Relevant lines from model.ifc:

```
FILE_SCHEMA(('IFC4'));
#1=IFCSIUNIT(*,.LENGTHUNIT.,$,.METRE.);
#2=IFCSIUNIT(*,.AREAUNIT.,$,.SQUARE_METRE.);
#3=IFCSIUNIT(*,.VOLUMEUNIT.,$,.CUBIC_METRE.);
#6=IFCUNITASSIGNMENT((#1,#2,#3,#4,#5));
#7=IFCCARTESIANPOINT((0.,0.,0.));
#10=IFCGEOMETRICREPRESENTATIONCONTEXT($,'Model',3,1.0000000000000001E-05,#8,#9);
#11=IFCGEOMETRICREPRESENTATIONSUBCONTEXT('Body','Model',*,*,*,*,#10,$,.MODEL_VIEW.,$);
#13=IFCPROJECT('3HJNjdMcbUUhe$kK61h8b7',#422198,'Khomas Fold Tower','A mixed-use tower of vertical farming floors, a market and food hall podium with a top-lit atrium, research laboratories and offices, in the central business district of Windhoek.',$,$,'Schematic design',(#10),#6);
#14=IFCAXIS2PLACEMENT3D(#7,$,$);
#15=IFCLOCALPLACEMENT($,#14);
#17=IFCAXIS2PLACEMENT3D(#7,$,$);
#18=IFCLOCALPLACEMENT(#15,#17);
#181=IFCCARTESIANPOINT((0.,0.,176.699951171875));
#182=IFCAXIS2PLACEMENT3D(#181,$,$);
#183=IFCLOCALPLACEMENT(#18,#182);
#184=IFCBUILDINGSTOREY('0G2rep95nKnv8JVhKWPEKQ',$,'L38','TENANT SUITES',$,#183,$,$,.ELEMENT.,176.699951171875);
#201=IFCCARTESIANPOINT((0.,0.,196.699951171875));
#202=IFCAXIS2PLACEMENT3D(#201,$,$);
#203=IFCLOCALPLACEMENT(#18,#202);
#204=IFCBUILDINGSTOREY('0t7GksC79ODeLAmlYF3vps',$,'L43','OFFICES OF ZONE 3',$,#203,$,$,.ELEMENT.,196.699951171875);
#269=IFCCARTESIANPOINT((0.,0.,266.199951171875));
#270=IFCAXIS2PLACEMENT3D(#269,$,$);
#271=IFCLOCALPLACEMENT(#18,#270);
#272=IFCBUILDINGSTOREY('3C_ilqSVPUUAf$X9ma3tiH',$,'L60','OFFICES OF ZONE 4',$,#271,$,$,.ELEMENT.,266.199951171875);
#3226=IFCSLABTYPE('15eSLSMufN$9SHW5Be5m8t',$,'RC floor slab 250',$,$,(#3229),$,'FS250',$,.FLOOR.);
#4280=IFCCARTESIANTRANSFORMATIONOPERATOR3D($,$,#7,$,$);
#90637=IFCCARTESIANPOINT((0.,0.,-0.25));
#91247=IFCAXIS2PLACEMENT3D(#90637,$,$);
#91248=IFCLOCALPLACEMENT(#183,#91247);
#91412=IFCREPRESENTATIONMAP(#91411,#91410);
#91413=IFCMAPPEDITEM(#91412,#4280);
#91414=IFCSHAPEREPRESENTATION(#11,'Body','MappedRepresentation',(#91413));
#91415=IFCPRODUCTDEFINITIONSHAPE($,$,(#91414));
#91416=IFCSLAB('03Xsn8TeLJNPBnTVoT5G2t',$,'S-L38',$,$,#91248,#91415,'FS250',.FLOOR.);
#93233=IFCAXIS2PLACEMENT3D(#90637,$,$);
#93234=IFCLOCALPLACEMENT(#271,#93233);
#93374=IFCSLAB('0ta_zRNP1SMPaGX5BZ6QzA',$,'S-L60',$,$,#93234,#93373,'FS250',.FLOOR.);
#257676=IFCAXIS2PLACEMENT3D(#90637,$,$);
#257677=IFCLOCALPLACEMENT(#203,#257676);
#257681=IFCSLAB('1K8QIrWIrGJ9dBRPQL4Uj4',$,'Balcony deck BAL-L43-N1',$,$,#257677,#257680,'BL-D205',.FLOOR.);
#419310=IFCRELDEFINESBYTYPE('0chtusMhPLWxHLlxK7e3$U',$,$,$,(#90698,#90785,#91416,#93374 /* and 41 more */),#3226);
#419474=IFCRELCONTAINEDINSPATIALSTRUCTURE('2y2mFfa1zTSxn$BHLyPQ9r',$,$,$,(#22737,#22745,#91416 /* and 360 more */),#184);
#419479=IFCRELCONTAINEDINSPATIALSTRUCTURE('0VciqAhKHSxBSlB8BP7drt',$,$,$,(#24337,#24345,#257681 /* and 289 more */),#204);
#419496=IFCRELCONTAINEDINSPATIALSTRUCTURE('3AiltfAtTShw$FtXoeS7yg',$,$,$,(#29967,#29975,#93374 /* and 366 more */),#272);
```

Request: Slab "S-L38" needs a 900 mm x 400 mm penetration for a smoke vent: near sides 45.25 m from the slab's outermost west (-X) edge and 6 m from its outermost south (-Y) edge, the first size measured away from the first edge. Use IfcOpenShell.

```python
import numpy as np
import ifcopenshell
import ifcopenshell.api.feature
import ifcopenshell.api.geometry
import ifcopenshell.api.root
import ifcopenshell.geom
import ifcopenshell.util.placement
import ifcopenshell.util.representation
import ifcopenshell.util.shape
import ifcopenshell.util.unit

model = ifcopenshell.open("model.ifc")
unit_scale = ifcopenshell.util.unit.calculate_unit_scale(model)
settings = ifcopenshell.geom.settings()


def volume(element):
    """Net volume in cubic metres, openings subtracted."""
    shape = ifcopenshell.geom.create_shape(settings, element)
    return ifcopenshell.util.shape.get_volume(shape.geometry)


slab = model.by_id(91416)
before = volume(slab)

# Extent in the slab's own axes, in metres. The edges named are its -X and -Y sides.
slab_shape = ifcopenshell.geom.create_shape(settings, slab)
vertices = ifcopenshell.util.shape.get_vertices(slab_shape.geometry)
x_min, y_min, bottom = vertices.min(axis=0)
top = vertices[:, 2].max()

opening = ifcopenshell.api.root.create_entity(model, ifc_class="IfcOpeningElement", name="Smoke vent opening", predefined_type="OPENING")
context = ifcopenshell.util.representation.get_context(model, "Model", "Body", "MODEL_VIEW")
width, depth = 0.9, 0.4
outline = [(0.0, 0.0), (width, 0.0), (width, depth), (0.0, depth), (0.0, 0.0)]
# Overshoot both faces by 50 mm so the cut is clean.
shape = ifcopenshell.api.geometry.add_slab_representation(
    model, context=context, depth=top - bottom + 0.1, polyline=outline
)
ifcopenshell.api.geometry.assign_representation(model, product=opening, representation=shape)

matrix = ifcopenshell.util.placement.get_local_placement(slab.ObjectPlacement)
matrix[:, 3] = matrix @ np.append(np.array([x_min + 45.25, y_min + 6, bottom - 0.05]) / unit_scale, 1.0)
ifcopenshell.api.geometry.edit_object_placement(model, product=opening, matrix=matrix, is_si=False)
ifcopenshell.api.feature.add_feature(model, feature=opening, element=slab)

after = volume(slab)

print(f"slab volume {before:.3f} -> {after:.3f} m3")

model.write("model_rev.ifc")
```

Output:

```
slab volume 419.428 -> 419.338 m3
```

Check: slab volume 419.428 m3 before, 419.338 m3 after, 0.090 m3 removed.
